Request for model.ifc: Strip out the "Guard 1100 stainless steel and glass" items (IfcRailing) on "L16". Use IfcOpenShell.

First a look at what the model holds.

```python
import ifcopenshell
import ifcopenshell.util.element

model = ifcopenshell.open("model.ifc")
print(model.schema)
storey = next(s for s in model.by_type("IfcBuildingStorey") if s.Name == "L16")
railings = [e for e in ifcopenshell.util.element.get_decomposition(storey) if e.is_a("IfcRailing")]
seen = {}
for e in railings:
    element_type = ifcopenshell.util.element.get_type(e)
    name = element_type.Name if element_type not in (None, e) else None
    seen[name] = seen.get(name, 0) + 1
for name, count in sorted(seen.items(), key=str):
    print(count, "x", name)
```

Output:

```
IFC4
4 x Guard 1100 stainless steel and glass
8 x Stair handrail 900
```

```python
import ifcopenshell
import ifcopenshell.api.root
import ifcopenshell.util.element

model = ifcopenshell.open("model.ifc")

storey = next(s for s in model.by_type("IfcBuildingStorey") if s.Name == "L16")
railings = [e for e in ifcopenshell.util.element.get_decomposition(storey) if e.is_a("IfcRailing")]
targets = [e for e in railings if (t := ifcopenshell.util.element.get_type(e)) not in (None, e) and t.Name == "Guard 1100 stainless steel and glass"]

for e in targets:
    ifcopenshell.api.root.remove_product(model, product=e)
print(len(targets), "removed")

model.write("model-out.ifc")
```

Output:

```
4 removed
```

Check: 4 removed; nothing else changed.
